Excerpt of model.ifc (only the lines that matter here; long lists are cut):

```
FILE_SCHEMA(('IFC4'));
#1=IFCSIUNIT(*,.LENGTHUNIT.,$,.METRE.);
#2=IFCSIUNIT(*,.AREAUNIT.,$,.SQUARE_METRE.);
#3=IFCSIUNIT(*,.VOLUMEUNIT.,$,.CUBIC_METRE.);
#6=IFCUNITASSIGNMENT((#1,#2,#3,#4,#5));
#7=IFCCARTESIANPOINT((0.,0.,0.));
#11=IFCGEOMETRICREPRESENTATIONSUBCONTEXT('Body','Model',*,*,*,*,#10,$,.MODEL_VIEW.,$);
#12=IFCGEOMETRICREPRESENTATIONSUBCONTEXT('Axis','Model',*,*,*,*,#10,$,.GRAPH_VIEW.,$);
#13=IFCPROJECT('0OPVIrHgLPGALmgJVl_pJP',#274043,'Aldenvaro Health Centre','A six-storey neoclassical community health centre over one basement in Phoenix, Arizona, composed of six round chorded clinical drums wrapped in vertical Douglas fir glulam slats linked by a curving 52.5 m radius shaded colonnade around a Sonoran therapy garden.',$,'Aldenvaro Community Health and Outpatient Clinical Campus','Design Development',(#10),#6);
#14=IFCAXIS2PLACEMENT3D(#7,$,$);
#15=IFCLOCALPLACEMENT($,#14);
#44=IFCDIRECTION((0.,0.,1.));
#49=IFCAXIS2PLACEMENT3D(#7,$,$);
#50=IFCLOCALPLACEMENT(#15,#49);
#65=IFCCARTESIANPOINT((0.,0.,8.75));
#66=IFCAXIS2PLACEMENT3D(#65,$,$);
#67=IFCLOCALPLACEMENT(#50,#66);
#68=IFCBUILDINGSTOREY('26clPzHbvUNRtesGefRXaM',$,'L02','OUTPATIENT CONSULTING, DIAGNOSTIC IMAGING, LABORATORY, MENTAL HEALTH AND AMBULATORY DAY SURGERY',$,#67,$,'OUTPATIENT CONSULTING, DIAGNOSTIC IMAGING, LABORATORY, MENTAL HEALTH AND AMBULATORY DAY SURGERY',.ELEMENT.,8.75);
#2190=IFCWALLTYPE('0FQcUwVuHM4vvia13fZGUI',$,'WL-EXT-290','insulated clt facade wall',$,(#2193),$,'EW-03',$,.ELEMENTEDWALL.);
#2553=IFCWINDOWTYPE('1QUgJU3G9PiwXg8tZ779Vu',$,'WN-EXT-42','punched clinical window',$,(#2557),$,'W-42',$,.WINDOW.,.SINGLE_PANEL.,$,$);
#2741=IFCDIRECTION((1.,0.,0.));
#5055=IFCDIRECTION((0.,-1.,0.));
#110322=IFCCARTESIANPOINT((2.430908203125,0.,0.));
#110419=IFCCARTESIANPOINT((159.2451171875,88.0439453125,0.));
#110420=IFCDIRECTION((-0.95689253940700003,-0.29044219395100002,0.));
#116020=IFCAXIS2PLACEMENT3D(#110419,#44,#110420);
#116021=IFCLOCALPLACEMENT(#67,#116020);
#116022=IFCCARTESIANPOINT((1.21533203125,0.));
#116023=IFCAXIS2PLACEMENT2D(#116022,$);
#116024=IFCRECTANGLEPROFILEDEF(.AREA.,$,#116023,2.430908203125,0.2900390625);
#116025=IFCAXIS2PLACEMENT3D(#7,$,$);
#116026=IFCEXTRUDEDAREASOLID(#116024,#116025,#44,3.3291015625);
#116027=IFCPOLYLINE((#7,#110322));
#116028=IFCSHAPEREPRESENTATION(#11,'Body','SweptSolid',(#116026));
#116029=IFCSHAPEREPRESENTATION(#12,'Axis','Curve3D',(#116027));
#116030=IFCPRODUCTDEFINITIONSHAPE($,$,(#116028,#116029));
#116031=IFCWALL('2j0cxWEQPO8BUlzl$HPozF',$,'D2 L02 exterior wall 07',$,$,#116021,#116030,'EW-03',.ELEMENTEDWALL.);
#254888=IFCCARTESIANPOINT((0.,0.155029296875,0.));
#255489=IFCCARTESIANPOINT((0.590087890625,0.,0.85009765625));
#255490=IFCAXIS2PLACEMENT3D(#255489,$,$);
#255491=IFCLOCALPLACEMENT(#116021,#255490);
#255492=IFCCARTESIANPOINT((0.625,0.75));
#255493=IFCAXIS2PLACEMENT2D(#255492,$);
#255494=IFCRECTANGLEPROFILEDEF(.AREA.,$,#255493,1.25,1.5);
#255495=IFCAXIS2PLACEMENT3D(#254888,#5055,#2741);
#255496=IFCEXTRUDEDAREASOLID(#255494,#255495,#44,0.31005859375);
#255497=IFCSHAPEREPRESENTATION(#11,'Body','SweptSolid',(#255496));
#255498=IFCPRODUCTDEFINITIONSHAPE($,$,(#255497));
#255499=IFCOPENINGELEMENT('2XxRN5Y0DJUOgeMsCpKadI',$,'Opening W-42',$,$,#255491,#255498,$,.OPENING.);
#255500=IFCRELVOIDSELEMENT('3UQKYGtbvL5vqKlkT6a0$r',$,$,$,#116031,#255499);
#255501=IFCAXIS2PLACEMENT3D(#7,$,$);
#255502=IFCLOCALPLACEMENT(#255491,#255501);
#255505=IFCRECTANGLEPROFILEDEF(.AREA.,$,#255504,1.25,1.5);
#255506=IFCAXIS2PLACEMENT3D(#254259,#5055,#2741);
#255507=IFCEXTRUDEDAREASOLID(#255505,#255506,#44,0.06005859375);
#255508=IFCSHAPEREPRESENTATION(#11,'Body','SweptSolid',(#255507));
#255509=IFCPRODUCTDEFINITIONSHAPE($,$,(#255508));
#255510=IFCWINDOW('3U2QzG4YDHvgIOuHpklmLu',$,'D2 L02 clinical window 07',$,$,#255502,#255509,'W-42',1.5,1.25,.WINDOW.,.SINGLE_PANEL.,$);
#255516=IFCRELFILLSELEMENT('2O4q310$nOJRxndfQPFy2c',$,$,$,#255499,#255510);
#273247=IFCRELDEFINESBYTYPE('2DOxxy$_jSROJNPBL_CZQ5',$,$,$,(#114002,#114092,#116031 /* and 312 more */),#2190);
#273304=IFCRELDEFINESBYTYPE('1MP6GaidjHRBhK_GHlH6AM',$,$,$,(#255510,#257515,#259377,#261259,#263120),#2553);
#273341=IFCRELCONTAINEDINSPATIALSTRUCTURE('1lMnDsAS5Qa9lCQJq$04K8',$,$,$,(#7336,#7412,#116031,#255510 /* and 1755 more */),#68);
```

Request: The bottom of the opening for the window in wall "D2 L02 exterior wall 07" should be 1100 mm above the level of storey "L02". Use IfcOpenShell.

```python
import numpy as np
import ifcopenshell
import ifcopenshell.api.geometry
import ifcopenshell.geom
import ifcopenshell.util.element
import ifcopenshell.util.placement
import ifcopenshell.util.shape
import ifcopenshell.util.unit

model = ifcopenshell.open("model.ifc")
unit_scale = ifcopenshell.util.unit.calculate_unit_scale(model)

window = model.by_guid("3U2QzG4YDHvgIOuHpklmLu")
opening = window.FillsVoids[0].RelatingOpeningElement
storey = ifcopenshell.util.element.get_container(window, ifc_class="IfcBuildingStorey")
level = ifcopenshell.util.placement.get_local_placement(storey.ObjectPlacement)[2, 3]

# The opening's origin need not be at the sill, so measure its lowest point.
shape = ifcopenshell.geom.create_shape(ifcopenshell.geom.settings(), opening)
bottom = ifcopenshell.util.shape.get_shape_bottom_elevation(shape, shape.geometry) / unit_scale
dz = level + 1.1 / unit_scale - bottom

shift = np.array([0.0, 0.0, dz])
# The window is placed relative to its opening, so it follows when the opening moves.
matrix = ifcopenshell.util.placement.get_local_placement(opening.ObjectPlacement)
matrix[:3, 3] += shift
ifcopenshell.api.geometry.edit_object_placement(
    model, product=opening, matrix=matrix, is_si=False, should_transform_children=True
)

print(f"moved by {dz * unit_scale:+.3f} m")

model.write("model-out.ifc")
```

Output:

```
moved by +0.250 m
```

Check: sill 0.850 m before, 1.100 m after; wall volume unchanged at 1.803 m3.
